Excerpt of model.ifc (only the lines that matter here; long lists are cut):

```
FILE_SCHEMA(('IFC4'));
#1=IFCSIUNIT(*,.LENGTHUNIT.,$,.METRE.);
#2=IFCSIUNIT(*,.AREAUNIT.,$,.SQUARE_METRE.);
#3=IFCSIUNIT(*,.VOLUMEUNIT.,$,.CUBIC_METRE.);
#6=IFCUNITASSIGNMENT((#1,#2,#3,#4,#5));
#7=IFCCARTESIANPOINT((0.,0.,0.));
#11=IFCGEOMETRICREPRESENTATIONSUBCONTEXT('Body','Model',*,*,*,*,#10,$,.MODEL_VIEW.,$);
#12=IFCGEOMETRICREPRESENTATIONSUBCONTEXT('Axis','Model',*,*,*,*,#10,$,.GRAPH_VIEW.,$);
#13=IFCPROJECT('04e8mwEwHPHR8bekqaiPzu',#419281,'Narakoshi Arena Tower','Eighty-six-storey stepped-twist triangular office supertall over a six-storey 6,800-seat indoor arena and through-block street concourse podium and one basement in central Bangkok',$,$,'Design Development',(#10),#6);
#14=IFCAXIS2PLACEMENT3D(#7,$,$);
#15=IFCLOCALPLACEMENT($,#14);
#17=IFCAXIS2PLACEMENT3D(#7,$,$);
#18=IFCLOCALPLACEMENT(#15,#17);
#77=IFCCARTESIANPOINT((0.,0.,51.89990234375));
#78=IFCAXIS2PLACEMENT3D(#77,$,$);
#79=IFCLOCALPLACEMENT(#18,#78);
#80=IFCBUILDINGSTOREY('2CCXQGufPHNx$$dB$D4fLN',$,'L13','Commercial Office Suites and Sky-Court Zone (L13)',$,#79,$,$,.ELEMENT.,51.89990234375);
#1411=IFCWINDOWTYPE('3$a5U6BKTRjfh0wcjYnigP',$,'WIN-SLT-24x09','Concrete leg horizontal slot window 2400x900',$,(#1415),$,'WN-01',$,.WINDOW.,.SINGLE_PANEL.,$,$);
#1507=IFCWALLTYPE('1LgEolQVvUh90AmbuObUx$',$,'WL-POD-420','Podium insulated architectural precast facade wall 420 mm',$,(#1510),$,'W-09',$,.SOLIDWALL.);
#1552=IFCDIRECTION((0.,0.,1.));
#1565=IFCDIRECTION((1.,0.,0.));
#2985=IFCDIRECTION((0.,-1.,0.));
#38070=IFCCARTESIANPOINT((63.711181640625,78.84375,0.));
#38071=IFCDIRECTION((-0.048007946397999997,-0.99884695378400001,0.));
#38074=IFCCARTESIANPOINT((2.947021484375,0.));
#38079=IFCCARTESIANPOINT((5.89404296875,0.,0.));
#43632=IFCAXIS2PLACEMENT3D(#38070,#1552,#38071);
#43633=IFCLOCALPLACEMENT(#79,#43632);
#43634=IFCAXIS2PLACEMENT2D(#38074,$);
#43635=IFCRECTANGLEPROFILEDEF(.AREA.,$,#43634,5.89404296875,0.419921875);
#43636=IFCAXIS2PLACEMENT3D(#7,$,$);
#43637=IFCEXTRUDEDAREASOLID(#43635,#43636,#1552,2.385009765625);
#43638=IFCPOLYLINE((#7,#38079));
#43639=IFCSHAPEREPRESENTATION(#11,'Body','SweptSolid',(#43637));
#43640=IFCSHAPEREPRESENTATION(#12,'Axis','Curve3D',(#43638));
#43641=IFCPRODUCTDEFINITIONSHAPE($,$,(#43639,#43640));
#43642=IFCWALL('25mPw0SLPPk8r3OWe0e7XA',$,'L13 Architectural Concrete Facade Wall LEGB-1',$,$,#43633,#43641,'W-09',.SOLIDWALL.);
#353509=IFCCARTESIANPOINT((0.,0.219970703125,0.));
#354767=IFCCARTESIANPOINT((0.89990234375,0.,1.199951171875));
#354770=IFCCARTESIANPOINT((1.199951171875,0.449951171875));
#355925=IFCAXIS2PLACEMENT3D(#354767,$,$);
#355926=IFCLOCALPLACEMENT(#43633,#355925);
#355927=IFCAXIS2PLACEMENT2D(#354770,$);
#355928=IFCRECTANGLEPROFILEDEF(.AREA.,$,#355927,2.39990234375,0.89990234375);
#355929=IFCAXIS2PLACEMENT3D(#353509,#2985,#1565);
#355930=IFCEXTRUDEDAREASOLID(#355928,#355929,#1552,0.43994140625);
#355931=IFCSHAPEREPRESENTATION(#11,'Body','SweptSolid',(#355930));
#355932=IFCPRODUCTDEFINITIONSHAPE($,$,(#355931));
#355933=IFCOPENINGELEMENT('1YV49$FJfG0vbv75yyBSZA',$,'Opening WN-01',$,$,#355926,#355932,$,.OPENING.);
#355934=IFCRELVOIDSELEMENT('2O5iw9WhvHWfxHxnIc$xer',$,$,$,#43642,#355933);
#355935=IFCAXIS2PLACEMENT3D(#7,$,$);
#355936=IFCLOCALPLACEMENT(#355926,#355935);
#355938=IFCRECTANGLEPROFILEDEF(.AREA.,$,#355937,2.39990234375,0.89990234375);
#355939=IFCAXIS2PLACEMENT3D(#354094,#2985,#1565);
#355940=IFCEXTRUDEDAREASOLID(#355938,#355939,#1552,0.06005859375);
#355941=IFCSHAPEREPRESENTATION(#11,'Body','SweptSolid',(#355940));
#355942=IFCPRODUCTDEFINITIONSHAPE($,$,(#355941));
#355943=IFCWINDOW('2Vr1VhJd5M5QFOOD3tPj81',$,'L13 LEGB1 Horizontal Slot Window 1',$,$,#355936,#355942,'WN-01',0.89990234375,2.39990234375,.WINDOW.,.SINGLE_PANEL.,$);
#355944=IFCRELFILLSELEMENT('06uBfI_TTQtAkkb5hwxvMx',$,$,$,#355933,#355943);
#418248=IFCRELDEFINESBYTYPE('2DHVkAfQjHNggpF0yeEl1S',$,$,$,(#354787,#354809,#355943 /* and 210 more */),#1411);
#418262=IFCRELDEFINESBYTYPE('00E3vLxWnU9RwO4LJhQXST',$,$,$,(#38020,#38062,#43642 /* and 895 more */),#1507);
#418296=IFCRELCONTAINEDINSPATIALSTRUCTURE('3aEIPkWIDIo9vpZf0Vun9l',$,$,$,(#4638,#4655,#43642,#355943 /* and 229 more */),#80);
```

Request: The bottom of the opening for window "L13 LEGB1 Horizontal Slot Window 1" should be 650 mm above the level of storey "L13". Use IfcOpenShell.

```python
import numpy as np
import ifcopenshell
import ifcopenshell.api.geometry
import ifcopenshell.geom
import ifcopenshell.util.element
import ifcopenshell.util.placement
import ifcopenshell.util.shape
import ifcopenshell.util.unit

model = ifcopenshell.open("model.ifc")
unit_scale = ifcopenshell.util.unit.calculate_unit_scale(model)

window = model.by_guid("2Vr1VhJd5M5QFOOD3tPj81")
opening = window.FillsVoids[0].RelatingOpeningElement
storey = ifcopenshell.util.element.get_container(window, ifc_class="IfcBuildingStorey")
level = ifcopenshell.util.placement.get_local_placement(storey.ObjectPlacement)[2, 3]

# The opening's origin need not be at the sill, so measure its lowest point.
shape = ifcopenshell.geom.create_shape(ifcopenshell.geom.settings(), opening)
bottom = ifcopenshell.util.shape.get_shape_bottom_elevation(shape, shape.geometry) / unit_scale
dz = level + 0.65 / unit_scale - bottom

shift = np.array([0.0, 0.0, dz])
# The window is placed relative to its opening, so it follows when the opening moves.
matrix = ifcopenshell.util.placement.get_local_placement(opening.ObjectPlacement)
matrix[:3, 3] += shift
ifcopenshell.api.geometry.edit_object_placement(
    model, product=opening, matrix=matrix, is_si=False, should_transform_children=True
)

print(f"moved by {dz * unit_scale:+.3f} m")

model.write("model_updated.ifc")
```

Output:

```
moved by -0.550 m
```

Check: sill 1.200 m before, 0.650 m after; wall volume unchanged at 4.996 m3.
